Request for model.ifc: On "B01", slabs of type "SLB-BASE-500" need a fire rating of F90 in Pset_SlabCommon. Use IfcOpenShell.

First a look at what the model holds.

```python
import ifcopenshell
import ifcopenshell.util.element

model = ifcopenshell.open("model.ifc")
print(model.schema)
storey = next(s for s in model.by_type("IfcBuildingStorey") if s.Name == "B01")
slabs = [e for e in ifcopenshell.util.element.get_decomposition(storey) if e.is_a("IfcSlab")]
seen = {}
for e in slabs:
    element_type = ifcopenshell.util.element.get_type(e)
    key = (element_type.Name if element_type != e and element_type else None, ifcopenshell.util.element.get_pset(e, "Pset_SlabCommon", "FireRating"))
    seen[key] = seen.get(key, 0) + 1
for (name, value), count in sorted(seen.items(), key=str):
    print(count, "x", name, "|", value)
```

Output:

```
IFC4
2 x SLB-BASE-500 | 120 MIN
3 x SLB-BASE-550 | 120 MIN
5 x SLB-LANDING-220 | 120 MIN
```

```python
import ifcopenshell
import ifcopenshell.api.pset
import ifcopenshell.util.element

model = ifcopenshell.open("model.ifc")

storey = next(s for s in model.by_type("IfcBuildingStorey") if s.Name == "B01")
slabs = [e for e in ifcopenshell.util.element.get_decomposition(storey) if e.is_a("IfcSlab")]

count = 0
for e in slabs:
    element_type = ifcopenshell.util.element.get_type(e)
    if element_type in (None, e) or element_type.Name != "SLB-BASE-500":
        continue
    # add_pset returns the element's existing set when there is one.
    pset = ifcopenshell.api.pset.add_pset(model, product=e, name="Pset_SlabCommon")
    ifcopenshell.api.pset.edit_pset(model, pset=pset, properties={"FireRating": "F90"})
    count += 1

print(count, "slabs updated")

model.write("model_edited.ifc")
```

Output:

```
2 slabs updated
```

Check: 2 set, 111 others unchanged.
